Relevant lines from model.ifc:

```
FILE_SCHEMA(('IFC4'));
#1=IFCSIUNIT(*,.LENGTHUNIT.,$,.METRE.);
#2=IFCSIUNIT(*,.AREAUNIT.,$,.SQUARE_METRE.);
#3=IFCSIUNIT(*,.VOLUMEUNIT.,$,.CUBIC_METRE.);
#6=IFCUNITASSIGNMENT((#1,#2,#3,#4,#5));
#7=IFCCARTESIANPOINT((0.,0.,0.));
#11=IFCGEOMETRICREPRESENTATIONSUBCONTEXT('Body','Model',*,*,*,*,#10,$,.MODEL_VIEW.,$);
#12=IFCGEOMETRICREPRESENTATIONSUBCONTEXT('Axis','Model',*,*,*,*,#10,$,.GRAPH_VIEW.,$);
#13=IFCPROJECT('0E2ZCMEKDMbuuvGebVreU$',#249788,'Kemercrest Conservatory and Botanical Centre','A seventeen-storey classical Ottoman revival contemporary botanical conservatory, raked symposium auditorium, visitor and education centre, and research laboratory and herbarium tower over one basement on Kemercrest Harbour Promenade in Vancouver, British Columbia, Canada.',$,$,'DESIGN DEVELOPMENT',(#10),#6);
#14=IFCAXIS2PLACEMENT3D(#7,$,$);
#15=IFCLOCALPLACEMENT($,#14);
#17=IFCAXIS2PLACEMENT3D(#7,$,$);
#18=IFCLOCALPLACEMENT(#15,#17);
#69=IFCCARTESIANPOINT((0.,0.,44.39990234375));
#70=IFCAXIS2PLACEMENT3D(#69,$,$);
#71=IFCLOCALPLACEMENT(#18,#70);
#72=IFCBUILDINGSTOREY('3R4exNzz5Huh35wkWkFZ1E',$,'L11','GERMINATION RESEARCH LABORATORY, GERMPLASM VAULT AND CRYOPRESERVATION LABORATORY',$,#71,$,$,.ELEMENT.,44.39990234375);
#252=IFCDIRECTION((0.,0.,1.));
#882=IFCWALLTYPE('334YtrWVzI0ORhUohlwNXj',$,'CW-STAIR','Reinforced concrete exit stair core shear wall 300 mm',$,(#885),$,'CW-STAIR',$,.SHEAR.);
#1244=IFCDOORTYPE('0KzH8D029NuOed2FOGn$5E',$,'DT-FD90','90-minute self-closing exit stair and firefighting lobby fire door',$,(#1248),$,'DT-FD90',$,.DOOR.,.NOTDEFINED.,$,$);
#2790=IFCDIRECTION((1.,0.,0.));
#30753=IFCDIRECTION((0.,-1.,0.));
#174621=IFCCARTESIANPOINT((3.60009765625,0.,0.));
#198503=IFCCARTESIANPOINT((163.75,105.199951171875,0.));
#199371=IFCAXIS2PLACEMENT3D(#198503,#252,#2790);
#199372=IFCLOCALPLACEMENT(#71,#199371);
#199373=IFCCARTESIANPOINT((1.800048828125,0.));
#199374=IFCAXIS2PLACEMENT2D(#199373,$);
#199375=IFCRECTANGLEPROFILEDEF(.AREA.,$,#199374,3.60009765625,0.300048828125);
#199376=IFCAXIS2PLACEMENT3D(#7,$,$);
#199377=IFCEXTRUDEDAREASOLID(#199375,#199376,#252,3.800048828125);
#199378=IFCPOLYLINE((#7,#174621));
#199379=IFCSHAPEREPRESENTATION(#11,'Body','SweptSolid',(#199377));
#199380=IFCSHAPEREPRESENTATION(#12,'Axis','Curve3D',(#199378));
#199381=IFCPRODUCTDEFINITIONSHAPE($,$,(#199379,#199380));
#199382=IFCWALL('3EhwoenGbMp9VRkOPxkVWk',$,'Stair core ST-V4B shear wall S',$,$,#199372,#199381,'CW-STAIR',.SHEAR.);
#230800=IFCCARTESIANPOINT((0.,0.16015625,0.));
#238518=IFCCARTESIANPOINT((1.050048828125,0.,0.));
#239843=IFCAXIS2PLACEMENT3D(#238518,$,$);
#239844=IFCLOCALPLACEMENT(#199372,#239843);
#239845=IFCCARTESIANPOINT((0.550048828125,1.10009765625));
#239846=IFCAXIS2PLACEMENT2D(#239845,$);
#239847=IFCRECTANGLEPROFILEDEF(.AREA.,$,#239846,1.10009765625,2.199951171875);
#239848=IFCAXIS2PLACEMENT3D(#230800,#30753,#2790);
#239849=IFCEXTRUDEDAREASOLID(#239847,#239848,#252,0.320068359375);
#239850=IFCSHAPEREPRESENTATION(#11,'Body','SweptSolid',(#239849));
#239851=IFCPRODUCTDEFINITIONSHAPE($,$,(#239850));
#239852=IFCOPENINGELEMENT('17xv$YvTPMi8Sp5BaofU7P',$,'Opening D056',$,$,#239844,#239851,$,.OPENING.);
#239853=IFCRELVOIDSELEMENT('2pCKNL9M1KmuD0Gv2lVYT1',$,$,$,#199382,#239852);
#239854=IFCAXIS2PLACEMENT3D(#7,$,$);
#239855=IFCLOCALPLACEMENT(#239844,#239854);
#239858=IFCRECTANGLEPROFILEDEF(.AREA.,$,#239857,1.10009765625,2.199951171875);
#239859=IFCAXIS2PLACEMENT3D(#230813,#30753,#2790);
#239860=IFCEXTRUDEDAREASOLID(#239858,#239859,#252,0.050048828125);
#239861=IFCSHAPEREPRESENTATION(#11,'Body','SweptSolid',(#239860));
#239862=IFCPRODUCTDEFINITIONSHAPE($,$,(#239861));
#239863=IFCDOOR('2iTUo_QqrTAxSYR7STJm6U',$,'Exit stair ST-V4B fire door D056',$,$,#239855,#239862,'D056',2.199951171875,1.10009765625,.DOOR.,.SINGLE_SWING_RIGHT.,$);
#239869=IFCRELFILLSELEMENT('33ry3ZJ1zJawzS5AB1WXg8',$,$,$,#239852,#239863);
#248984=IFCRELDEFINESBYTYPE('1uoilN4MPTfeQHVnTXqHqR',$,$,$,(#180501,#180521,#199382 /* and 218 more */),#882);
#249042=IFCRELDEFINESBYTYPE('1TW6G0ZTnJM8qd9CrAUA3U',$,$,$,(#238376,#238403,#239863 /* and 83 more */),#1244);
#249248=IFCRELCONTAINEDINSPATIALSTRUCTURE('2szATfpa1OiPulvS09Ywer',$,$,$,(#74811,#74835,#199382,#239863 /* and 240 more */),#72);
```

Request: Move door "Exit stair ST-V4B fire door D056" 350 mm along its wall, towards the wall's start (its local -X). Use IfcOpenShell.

```python
import ifcopenshell
import ifcopenshell.api.geometry
import ifcopenshell.util.placement

model = ifcopenshell.open("model.ifc")

door = model.by_guid("2iTUo_QqrTAxSYR7STJm6U")
opening = door.FillsVoids[0].RelatingOpeningElement
wall = opening.VoidsElements[0].RelatingBuildingElement

wall_matrix = ifcopenshell.util.placement.get_local_placement(wall.ObjectPlacement)
shift = wall_matrix[:3, 0] * -0.35
before = ifcopenshell.util.placement.get_local_placement(door.ObjectPlacement)[:3, 3].copy()

# The door is placed relative to its opening, so it follows when the opening moves.
matrix = ifcopenshell.util.placement.get_local_placement(opening.ObjectPlacement)
matrix[:3, 3] += shift
ifcopenshell.api.geometry.edit_object_placement(
    model, product=opening, matrix=matrix, is_si=False, should_transform_children=True
)

after = ifcopenshell.util.placement.get_local_placement(door.ObjectPlacement)[:3, 3]
print("door moved by", (after - before).round(3) + 0.0)

model.write("model-out.ifc")
```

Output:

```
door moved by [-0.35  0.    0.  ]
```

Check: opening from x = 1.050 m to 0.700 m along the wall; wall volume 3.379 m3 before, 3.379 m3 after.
